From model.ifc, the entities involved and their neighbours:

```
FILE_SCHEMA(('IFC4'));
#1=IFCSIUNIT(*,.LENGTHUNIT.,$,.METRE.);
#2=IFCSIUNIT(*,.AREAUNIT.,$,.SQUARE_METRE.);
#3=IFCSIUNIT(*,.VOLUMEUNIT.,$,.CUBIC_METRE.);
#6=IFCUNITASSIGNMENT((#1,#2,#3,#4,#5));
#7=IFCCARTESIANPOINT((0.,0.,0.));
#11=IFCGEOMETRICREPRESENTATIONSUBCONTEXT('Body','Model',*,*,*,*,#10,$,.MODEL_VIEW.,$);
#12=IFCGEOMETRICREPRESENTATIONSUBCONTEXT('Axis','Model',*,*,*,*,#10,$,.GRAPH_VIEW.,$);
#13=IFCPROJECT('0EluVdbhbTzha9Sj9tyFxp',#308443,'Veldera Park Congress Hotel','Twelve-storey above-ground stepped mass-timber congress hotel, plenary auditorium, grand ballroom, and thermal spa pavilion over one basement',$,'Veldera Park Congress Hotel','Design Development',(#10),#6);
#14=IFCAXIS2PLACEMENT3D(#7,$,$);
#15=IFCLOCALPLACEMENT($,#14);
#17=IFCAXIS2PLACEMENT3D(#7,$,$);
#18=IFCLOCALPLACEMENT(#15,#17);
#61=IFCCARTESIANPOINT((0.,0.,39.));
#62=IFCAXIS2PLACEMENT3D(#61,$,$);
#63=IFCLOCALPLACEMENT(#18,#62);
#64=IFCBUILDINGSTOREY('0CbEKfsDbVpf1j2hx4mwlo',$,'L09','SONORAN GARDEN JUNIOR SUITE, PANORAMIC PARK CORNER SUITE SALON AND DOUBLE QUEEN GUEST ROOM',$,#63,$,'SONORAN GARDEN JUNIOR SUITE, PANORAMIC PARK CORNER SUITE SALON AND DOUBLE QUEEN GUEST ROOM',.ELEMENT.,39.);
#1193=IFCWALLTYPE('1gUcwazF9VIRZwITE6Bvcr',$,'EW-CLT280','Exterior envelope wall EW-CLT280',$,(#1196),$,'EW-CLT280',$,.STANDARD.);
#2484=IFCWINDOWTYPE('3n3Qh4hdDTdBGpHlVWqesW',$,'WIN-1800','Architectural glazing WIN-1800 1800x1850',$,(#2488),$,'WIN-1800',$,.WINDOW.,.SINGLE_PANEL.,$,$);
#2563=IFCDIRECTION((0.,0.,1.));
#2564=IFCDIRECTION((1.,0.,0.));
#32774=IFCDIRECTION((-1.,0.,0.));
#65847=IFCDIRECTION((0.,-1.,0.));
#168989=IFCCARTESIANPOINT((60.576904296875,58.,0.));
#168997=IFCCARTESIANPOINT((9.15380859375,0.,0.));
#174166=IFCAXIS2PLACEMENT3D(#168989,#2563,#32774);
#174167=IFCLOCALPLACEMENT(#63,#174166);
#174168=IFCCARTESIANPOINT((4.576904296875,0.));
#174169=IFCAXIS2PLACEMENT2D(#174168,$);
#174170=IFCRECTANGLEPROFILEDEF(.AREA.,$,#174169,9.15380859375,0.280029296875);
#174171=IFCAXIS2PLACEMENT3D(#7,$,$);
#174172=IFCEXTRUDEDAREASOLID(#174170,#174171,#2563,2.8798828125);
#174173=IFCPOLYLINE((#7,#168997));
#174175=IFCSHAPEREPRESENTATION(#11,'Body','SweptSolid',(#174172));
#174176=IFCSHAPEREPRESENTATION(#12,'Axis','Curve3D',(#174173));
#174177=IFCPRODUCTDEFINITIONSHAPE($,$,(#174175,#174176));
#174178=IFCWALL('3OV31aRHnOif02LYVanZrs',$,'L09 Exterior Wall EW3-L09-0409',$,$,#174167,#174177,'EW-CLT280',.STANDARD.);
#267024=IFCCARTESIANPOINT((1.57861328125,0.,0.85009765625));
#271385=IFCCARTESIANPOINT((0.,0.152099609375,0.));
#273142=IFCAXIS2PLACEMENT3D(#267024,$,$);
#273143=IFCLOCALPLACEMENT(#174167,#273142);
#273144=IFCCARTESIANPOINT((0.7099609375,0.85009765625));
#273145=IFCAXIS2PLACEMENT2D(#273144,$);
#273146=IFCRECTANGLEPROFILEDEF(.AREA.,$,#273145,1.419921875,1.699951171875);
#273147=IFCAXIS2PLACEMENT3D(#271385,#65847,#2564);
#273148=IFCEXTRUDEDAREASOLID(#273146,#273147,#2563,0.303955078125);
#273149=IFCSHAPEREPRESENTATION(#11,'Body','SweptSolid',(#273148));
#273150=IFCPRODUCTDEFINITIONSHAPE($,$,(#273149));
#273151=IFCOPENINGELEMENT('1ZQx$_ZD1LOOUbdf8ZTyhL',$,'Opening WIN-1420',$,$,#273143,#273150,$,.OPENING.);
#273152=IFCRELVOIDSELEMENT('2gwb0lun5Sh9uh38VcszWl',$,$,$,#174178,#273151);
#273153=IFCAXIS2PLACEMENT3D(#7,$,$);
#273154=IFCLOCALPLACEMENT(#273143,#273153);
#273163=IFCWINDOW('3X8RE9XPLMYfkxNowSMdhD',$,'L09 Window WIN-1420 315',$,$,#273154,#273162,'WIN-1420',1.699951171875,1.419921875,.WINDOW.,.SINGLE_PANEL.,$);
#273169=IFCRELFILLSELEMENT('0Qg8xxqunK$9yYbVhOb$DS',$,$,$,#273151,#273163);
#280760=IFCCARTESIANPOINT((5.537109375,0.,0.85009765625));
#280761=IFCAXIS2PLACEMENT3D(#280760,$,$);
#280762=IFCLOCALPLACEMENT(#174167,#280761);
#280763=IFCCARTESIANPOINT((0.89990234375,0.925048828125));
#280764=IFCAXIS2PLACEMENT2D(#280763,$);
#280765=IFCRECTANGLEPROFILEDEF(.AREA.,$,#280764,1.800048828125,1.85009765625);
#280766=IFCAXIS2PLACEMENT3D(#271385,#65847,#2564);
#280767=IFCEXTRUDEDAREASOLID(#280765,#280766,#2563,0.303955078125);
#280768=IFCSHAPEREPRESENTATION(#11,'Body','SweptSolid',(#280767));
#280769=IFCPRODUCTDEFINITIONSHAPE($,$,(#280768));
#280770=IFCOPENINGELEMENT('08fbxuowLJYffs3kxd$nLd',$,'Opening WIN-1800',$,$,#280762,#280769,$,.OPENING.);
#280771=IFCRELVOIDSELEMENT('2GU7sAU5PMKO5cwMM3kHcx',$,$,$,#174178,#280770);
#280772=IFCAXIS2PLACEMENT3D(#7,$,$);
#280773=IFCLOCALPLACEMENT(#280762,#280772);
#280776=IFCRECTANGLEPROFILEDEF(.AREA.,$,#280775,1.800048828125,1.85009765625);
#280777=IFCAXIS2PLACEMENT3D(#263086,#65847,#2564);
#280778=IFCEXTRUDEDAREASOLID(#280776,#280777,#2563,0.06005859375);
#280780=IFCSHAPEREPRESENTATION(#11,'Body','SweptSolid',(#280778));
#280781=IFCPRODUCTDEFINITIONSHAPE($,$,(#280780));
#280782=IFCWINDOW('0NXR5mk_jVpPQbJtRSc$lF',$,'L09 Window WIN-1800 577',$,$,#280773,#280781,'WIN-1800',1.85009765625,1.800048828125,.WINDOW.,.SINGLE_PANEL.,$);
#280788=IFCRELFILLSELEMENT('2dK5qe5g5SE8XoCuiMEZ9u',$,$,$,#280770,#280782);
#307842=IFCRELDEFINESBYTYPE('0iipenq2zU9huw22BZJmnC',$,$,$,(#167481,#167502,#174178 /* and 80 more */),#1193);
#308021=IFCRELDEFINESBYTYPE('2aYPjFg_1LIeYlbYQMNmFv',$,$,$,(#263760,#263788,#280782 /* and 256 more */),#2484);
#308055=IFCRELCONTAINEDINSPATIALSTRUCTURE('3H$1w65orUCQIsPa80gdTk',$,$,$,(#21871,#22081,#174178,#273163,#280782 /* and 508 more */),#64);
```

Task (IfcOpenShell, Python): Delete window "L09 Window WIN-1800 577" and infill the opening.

```python
import ifcopenshell
import ifcopenshell.api.feature
import ifcopenshell.api.root
import ifcopenshell.geom
import ifcopenshell.util.shape

model = ifcopenshell.open("model.ifc")
settings = ifcopenshell.geom.settings()


def volume(element):
    """Net volume in cubic metres, openings subtracted."""
    shape = ifcopenshell.geom.create_shape(settings, element)
    return ifcopenshell.util.shape.get_volume(shape.geometry)


window = model.by_guid("0NXR5mk_jVpPQbJtRSc$lF")
opening = window.FillsVoids[0].RelatingOpeningElement
wall = opening.VoidsElements[0].RelatingBuildingElement
before = volume(wall)

ifcopenshell.api.root.remove_product(model, product=window)
ifcopenshell.api.feature.remove_feature(model, feature=opening)

after = volume(wall)

print(f"wall volume {before:.3f} -> {after:.3f} m3")

model.write("model_updated.ifc")
```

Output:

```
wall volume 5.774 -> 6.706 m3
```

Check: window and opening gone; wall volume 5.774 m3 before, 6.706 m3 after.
